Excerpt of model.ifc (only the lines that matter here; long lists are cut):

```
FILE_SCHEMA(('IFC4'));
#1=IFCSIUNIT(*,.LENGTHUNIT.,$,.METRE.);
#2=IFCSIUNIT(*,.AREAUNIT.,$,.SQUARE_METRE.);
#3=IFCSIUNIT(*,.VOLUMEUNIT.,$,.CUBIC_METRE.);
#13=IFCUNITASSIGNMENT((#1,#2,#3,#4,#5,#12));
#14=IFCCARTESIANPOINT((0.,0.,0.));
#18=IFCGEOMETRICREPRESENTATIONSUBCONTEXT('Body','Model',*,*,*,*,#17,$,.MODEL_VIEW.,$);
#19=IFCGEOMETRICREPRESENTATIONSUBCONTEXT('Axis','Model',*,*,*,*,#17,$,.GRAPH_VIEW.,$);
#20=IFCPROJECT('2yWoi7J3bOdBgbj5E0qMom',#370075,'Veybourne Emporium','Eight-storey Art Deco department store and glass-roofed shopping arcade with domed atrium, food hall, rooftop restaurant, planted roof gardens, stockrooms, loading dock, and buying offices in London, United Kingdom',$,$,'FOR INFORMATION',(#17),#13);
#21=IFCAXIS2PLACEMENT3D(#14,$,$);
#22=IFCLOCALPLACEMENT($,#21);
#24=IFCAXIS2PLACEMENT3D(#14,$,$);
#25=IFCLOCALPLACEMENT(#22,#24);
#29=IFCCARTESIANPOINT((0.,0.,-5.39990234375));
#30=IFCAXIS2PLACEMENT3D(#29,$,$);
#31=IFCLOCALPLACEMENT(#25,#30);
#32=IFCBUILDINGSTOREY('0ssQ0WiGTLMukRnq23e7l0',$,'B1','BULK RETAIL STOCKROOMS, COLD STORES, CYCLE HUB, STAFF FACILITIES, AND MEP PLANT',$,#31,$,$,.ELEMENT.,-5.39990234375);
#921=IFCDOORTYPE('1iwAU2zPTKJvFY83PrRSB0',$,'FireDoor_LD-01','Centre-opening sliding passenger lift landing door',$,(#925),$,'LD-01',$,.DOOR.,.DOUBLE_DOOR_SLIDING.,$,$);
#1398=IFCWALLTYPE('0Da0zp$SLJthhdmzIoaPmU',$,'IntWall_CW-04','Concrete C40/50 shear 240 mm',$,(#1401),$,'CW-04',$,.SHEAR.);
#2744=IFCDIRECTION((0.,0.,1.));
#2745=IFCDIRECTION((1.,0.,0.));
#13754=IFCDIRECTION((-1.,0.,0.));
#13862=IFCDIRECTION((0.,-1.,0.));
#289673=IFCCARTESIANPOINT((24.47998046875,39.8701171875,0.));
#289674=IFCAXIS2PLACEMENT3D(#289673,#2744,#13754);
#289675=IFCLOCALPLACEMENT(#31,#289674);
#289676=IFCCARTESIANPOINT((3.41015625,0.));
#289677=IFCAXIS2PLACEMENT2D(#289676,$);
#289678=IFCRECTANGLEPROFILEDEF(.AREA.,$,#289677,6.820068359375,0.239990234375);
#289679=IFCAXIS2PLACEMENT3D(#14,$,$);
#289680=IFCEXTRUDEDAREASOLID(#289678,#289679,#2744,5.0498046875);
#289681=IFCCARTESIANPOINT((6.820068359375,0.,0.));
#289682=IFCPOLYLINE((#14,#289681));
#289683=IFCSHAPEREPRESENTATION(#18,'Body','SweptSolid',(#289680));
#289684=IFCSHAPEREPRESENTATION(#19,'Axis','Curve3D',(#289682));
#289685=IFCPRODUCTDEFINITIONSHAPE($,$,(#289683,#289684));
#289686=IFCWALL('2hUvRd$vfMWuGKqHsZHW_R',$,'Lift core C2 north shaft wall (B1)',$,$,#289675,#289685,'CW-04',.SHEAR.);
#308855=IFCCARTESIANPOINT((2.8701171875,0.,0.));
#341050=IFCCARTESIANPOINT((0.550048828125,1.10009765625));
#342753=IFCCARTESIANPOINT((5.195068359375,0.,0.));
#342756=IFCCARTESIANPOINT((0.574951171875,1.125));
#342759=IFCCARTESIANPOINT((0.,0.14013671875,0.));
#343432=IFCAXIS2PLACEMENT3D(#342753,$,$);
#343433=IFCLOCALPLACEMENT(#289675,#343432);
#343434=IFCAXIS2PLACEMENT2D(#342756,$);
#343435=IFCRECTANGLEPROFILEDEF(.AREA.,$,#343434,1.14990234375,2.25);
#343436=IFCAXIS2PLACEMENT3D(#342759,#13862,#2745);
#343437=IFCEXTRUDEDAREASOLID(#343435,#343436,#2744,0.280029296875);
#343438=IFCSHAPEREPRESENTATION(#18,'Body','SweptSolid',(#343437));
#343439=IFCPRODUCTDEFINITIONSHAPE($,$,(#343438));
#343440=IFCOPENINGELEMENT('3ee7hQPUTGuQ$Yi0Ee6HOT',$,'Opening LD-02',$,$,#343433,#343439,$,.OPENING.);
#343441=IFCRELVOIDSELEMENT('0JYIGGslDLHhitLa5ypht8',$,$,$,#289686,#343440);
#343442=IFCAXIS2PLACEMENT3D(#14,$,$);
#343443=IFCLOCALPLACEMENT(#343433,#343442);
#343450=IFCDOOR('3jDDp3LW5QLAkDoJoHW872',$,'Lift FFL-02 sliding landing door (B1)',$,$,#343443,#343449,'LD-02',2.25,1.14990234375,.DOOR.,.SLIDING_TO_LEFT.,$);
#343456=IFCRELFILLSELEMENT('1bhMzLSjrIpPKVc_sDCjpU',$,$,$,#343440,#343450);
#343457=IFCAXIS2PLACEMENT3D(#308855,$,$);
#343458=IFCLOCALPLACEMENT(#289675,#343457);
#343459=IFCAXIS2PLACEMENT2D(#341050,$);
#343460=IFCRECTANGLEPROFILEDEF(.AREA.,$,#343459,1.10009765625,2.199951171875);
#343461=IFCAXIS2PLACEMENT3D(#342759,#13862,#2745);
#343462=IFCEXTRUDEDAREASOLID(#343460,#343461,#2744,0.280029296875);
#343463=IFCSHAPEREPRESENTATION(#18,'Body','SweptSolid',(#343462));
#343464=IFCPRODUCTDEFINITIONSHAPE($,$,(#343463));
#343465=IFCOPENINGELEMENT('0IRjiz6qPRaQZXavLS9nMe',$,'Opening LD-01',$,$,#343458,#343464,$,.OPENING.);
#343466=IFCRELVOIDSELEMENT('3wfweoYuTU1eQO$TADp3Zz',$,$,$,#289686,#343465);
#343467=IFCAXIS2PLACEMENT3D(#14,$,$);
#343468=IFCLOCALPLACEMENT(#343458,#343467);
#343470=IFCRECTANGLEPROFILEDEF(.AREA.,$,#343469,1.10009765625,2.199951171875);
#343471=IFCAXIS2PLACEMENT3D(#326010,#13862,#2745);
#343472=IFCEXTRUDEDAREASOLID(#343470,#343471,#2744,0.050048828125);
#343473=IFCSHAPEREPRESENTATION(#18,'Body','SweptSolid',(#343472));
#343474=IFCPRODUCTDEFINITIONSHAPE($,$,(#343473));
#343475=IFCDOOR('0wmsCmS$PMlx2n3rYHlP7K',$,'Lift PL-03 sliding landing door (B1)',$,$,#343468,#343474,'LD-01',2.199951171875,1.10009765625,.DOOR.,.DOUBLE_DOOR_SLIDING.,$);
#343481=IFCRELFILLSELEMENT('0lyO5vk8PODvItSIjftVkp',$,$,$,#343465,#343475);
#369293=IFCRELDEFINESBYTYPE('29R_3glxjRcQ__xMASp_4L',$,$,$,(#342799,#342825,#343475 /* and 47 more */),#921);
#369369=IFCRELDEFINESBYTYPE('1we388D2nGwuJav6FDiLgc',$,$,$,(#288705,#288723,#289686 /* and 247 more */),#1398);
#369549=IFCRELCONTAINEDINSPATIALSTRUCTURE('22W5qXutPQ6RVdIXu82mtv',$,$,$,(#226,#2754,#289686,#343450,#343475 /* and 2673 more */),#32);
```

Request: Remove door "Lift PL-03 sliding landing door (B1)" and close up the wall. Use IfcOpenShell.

```python
import ifcopenshell
import ifcopenshell.api.feature
import ifcopenshell.api.root
import ifcopenshell.geom
import ifcopenshell.util.shape

model = ifcopenshell.open("model.ifc")
settings = ifcopenshell.geom.settings()


def volume(element):
    """Net volume in cubic metres, openings subtracted."""
    shape = ifcopenshell.geom.create_shape(settings, element)
    return ifcopenshell.util.shape.get_volume(shape.geometry)


door = model.by_guid("0wmsCmS$PMlx2n3rYHlP7K")
opening = door.FillsVoids[0].RelatingOpeningElement
wall = opening.VoidsElements[0].RelatingBuildingElement
before = volume(wall)

ifcopenshell.api.root.remove_product(model, product=door)
ifcopenshell.api.feature.remove_feature(model, feature=opening)

after = volume(wall)

print(f"wall volume {before:.3f} -> {after:.3f} m3")

model.write("model_edited.ifc")
```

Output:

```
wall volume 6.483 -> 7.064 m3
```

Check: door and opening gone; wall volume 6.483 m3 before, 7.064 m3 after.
